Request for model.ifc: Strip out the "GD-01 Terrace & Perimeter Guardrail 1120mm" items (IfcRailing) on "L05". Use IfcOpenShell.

First a look at what the model holds.

```python
import ifcopenshell
import ifcopenshell.util.element

model = ifcopenshell.open("model.ifc")
print(model.schema)
storey = next(s for s in model.by_type("IfcBuildingStorey") if s.Name == "L05")
railings = [e for e in ifcopenshell.util.element.get_decomposition(storey) if e.is_a("IfcRailing")]
seen = {}
for e in railings:
    element_type = ifcopenshell.util.element.get_type(e)
    name = element_type.Name if element_type not in (None, e) else None
    seen[name] = seen.get(name, 0) + 1
for name, count in sorted(seen.items(), key=str):
    print(count, "x", name)
```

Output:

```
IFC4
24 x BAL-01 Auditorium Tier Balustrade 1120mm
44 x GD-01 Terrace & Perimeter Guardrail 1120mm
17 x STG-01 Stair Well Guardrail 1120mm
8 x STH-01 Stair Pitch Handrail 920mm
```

```python
import ifcopenshell
import ifcopenshell.api.root
import ifcopenshell.util.element

model = ifcopenshell.open("model.ifc")

storey = next(s for s in model.by_type("IfcBuildingStorey") if s.Name == "L05")
railings = [e for e in ifcopenshell.util.element.get_decomposition(storey) if e.is_a("IfcRailing")]
targets = [e for e in railings if (t := ifcopenshell.util.element.get_type(e)) not in (None, e) and t.Name == "GD-01 Terrace & Perimeter Guardrail 1120mm"]

for e in targets:
    ifcopenshell.api.root.remove_product(model, product=e)
print(len(targets), "removed")

model.write("model_edited.ifc")
```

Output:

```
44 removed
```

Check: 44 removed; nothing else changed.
